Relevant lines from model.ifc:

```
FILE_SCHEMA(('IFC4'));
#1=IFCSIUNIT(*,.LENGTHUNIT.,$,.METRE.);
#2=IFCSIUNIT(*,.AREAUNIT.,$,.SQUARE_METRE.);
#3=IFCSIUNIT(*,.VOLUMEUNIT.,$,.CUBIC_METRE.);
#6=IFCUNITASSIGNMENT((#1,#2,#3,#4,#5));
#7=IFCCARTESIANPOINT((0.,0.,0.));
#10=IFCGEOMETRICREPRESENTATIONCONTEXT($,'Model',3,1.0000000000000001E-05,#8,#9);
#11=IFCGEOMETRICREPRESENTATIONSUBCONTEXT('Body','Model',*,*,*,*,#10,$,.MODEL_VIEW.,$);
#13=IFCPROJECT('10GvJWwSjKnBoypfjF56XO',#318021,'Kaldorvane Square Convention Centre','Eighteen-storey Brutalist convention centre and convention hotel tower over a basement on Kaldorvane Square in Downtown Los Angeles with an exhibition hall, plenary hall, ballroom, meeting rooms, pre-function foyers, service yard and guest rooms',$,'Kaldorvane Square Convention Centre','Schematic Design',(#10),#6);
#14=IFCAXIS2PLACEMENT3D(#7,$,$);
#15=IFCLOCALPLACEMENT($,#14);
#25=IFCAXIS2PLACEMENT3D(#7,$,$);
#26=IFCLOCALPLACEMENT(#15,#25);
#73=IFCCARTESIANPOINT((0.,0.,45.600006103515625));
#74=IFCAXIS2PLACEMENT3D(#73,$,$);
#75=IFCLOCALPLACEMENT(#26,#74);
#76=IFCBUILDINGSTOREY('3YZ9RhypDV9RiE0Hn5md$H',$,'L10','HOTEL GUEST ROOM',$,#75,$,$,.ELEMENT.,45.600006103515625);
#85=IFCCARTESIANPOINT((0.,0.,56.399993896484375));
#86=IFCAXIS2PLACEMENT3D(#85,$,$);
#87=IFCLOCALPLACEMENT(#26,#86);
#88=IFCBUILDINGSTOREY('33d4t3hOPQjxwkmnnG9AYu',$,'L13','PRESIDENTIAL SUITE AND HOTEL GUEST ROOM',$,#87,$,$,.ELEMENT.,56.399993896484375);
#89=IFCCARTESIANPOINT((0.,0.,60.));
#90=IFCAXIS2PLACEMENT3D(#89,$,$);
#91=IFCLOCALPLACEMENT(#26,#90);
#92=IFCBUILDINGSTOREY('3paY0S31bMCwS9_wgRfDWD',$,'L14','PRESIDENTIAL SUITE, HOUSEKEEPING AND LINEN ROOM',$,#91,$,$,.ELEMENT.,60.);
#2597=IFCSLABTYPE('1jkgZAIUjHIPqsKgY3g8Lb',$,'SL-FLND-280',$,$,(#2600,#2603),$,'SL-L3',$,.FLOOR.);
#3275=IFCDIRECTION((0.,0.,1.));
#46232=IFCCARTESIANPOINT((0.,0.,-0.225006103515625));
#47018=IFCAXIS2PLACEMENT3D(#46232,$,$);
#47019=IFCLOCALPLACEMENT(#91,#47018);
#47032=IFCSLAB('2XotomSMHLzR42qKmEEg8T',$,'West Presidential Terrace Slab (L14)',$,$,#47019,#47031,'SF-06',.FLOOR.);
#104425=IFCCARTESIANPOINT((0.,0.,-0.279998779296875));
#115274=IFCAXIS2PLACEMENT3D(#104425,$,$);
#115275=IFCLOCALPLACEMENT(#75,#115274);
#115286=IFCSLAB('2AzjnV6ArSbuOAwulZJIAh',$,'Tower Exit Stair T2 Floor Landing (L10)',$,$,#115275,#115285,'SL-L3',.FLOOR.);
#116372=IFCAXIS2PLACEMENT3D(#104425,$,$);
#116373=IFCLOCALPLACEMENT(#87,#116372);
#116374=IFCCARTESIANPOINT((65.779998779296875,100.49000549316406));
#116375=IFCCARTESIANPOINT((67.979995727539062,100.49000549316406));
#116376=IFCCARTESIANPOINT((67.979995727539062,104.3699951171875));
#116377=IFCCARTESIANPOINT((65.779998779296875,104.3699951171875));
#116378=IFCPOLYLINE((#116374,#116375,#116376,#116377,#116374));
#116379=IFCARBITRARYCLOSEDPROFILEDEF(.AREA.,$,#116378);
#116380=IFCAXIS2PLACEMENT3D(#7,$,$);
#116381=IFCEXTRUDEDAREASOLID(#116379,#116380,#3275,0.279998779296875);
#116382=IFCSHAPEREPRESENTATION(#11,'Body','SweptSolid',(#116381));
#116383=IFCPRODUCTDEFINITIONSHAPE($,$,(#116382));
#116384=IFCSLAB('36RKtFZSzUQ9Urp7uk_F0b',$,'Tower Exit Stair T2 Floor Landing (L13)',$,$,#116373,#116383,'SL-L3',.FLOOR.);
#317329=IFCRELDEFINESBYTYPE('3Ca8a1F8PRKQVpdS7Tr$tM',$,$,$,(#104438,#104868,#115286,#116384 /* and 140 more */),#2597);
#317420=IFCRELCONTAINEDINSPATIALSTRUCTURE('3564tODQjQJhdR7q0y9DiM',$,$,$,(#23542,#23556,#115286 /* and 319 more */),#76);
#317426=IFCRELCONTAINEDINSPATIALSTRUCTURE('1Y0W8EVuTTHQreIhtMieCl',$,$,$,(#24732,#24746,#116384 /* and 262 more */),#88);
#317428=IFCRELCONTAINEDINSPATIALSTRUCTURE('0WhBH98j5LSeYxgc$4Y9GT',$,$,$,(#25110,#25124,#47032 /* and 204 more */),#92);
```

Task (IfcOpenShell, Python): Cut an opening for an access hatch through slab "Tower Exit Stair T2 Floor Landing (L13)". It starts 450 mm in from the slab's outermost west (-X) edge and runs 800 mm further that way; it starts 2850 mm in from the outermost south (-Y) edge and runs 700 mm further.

```python
import numpy as np
import ifcopenshell
import ifcopenshell.api.feature
import ifcopenshell.api.geometry
import ifcopenshell.api.root
import ifcopenshell.geom
import ifcopenshell.util.placement
import ifcopenshell.util.representation
import ifcopenshell.util.shape
import ifcopenshell.util.unit

model = ifcopenshell.open("model.ifc")
unit_scale = ifcopenshell.util.unit.calculate_unit_scale(model)
settings = ifcopenshell.geom.settings()


def volume(element):
    """Net volume in cubic metres, openings subtracted."""
    shape = ifcopenshell.geom.create_shape(settings, element)
    return ifcopenshell.util.shape.get_volume(shape.geometry)


slab = model.by_id(116384)
before = volume(slab)

# Extent in the slab's own axes, in metres. The edges named are its -X and -Y sides.
slab_shape = ifcopenshell.geom.create_shape(settings, slab)
vertices = ifcopenshell.util.shape.get_vertices(slab_shape.geometry)
x_min, y_min, bottom = vertices.min(axis=0)
top = vertices[:, 2].max()

opening = ifcopenshell.api.root.create_entity(model, ifc_class="IfcOpeningElement", name="Access hatch opening", predefined_type="OPENING")
context = ifcopenshell.util.representation.get_context(model, "Model", "Body", "MODEL_VIEW")
width, depth = 0.8, 0.7
outline = [(0.0, 0.0), (width, 0.0), (width, depth), (0.0, depth), (0.0, 0.0)]
# Overshoot both faces by 50 mm so the cut is clean.
shape = ifcopenshell.api.geometry.add_slab_representation(
    model, context=context, depth=top - bottom + 0.1, polyline=outline
)
ifcopenshell.api.geometry.assign_representation(model, product=opening, representation=shape)

matrix = ifcopenshell.util.placement.get_local_placement(slab.ObjectPlacement)
matrix[:, 3] = matrix @ np.append(np.array([x_min + 0.45, y_min + 2.85, bottom - 0.05]) / unit_scale, 1.0)
ifcopenshell.api.geometry.edit_object_placement(model, product=opening, matrix=matrix, is_si=False)
ifcopenshell.api.feature.add_feature(model, feature=opening, element=slab)

after = volume(slab)

print(f"slab volume {before:.3f} -> {after:.3f} m3")

model.write("model-out.ifc")
```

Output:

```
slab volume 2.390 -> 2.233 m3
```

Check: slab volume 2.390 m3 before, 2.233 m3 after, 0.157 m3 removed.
